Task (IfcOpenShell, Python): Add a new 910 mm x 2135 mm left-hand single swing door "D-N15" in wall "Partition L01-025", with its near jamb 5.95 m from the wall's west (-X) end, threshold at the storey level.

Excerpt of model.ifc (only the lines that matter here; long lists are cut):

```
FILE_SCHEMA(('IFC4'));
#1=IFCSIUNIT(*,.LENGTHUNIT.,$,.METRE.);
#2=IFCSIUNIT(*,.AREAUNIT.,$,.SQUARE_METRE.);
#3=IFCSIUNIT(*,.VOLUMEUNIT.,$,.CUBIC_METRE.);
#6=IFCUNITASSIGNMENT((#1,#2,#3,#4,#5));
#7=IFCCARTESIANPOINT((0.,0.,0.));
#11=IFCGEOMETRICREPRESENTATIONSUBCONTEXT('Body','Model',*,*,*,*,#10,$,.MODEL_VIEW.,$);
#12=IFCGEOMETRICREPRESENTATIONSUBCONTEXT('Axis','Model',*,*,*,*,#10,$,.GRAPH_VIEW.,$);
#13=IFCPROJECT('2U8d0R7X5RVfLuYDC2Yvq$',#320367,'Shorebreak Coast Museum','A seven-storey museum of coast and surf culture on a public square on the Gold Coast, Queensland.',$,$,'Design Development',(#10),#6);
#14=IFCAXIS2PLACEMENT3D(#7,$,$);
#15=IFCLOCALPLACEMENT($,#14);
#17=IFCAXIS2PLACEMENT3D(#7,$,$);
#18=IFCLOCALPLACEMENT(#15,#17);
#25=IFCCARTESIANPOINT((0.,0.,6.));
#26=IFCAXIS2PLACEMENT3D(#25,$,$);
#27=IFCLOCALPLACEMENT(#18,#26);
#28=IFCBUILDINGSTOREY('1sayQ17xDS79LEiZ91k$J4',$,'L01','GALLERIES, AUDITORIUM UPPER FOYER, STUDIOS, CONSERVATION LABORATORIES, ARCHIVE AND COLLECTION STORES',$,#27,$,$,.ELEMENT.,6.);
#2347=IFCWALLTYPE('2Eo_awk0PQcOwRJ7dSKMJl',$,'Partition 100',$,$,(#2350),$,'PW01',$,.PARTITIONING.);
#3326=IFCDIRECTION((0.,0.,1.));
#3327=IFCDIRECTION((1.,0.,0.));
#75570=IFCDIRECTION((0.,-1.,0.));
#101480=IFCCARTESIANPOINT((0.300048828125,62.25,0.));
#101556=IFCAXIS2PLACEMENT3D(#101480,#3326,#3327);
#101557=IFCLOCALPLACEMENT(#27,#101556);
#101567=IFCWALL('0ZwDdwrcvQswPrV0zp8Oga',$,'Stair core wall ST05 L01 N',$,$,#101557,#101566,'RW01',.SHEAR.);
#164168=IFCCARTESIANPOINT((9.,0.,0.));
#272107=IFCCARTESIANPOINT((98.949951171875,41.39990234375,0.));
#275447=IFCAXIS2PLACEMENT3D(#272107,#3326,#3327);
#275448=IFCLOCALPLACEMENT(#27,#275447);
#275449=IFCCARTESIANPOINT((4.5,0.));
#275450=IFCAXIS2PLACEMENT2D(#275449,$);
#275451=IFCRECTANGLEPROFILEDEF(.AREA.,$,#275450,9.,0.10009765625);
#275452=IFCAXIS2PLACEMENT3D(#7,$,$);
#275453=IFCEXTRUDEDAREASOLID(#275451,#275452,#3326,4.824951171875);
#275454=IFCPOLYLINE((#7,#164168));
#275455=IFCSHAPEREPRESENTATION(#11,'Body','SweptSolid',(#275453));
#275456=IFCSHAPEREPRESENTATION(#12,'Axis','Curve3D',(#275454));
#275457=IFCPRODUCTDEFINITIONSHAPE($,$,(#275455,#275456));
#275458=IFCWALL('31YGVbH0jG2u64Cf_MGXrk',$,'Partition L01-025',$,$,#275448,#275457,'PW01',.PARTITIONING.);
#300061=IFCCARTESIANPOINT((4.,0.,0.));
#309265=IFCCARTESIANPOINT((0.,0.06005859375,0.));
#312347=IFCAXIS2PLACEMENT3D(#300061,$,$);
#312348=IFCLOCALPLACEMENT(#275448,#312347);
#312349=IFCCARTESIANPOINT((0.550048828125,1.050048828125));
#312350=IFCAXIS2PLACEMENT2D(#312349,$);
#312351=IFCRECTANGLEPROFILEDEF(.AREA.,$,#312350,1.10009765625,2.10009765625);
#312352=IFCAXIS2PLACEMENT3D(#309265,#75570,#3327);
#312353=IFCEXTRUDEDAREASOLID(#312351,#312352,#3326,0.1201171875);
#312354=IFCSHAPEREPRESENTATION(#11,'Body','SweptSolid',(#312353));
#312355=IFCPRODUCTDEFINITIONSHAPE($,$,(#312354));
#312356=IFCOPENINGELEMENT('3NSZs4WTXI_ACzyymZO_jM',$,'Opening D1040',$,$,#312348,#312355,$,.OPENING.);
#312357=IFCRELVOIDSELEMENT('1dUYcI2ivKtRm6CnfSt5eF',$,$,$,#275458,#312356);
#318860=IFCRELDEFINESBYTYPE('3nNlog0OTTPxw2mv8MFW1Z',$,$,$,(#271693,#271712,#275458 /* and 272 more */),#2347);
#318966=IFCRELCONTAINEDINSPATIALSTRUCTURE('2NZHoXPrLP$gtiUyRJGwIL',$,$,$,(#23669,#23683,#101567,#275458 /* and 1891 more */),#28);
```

```python
import numpy as np
import ifcopenshell
import ifcopenshell.api.feature
import ifcopenshell.api.geometry
import ifcopenshell.api.root
import ifcopenshell.api.spatial
import ifcopenshell.geom
import ifcopenshell.util.element
import ifcopenshell.util.placement
import ifcopenshell.util.representation
import ifcopenshell.util.shape
import ifcopenshell.util.unit

model = ifcopenshell.open("model.ifc")
unit_scale = ifcopenshell.util.unit.calculate_unit_scale(model)
settings = ifcopenshell.geom.settings()


def volume(element):
    """Net volume in cubic metres, openings subtracted."""
    shape = ifcopenshell.geom.create_shape(settings, element)
    return ifcopenshell.util.shape.get_volume(shape.geometry)


wall = model.by_guid("31YGVbH0jG2u64Cf_MGXrk")
storey = ifcopenshell.util.element.get_container(wall, ifc_class="IfcBuildingStorey")
context = ifcopenshell.util.representation.get_context(model, "Model", "Body", "MODEL_VIEW")
before = volume(wall)

width, height, from_end, sill = 0.91, 2.135, 5.95, 0.0  # metres

# The wall runs along its own X axis, and the end named is its -X end.
wall_shape = ifcopenshell.geom.create_shape(settings, wall)
x, y, z = ifcopenshell.util.shape.get_vertices(wall_shape.geometry).T
start = x.min() + from_end
face, thickness = float(y.min()), float(y.max() - y.min())
wall_matrix = ifcopenshell.util.placement.get_local_placement(wall.ObjectPlacement)
level = ifcopenshell.util.placement.get_local_placement(storey.ObjectPlacement)[2, 3]


def in_wall(x, y):
    """Placement at x, y metres in the wall's axes, at sill height."""
    matrix = wall_matrix.copy()
    matrix[:, 3] = wall_matrix @ np.array([x / unit_scale, y / unit_scale, 0.0, 1.0])
    matrix[2, 3] = level + sill / unit_scale
    return matrix


# Opening: a box that overshoots both wall faces by 50 mm.
opening = ifcopenshell.api.root.create_entity(model, ifc_class="IfcOpeningElement", predefined_type="OPENING")
box = ifcopenshell.api.geometry.add_wall_representation(
    model, context=context, length=width, height=height, thickness=thickness + 0.1
)
ifcopenshell.api.geometry.assign_representation(model, product=opening, representation=box)
ifcopenshell.api.geometry.edit_object_placement(model, product=opening, matrix=in_wall(start, face - 0.05), is_si=False)
ifcopenshell.api.feature.add_feature(model, feature=opening, element=wall)

door = ifcopenshell.api.root.create_entity(model, ifc_class="IfcDoor", name="D-N15", predefined_type="DOOR")
door.OverallWidth, door.OverallHeight = width / unit_scale, height / unit_scale
door.OperationType = "SINGLE_SWING_LEFT"
body = ifcopenshell.api.geometry.add_door_representation(
    model,
    context=context,
    overall_width=door.OverallWidth,
    overall_height=door.OverallHeight,
    operation_type="SINGLE_SWING_LEFT",
    lining_properties={"LiningDepth": thickness / unit_scale, "ThresholdDepth": thickness / unit_scale},
)
ifcopenshell.api.geometry.assign_representation(model, product=door, representation=body)
ifcopenshell.api.spatial.assign_container(model, products=[door], relating_structure=storey)
ifcopenshell.api.feature.add_filling(model, opening=opening, element=door)

# The lining spans the wall, so the door starts at the wall face.
ifcopenshell.api.geometry.edit_object_placement(model, product=door, matrix=in_wall(start, face), is_si=False)

after = volume(wall)

print(f"wall volume {before:.3f} -> {after:.3f} m3")

model.write("model_edited.ifc")
```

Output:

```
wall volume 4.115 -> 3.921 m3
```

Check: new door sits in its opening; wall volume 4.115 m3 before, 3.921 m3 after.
